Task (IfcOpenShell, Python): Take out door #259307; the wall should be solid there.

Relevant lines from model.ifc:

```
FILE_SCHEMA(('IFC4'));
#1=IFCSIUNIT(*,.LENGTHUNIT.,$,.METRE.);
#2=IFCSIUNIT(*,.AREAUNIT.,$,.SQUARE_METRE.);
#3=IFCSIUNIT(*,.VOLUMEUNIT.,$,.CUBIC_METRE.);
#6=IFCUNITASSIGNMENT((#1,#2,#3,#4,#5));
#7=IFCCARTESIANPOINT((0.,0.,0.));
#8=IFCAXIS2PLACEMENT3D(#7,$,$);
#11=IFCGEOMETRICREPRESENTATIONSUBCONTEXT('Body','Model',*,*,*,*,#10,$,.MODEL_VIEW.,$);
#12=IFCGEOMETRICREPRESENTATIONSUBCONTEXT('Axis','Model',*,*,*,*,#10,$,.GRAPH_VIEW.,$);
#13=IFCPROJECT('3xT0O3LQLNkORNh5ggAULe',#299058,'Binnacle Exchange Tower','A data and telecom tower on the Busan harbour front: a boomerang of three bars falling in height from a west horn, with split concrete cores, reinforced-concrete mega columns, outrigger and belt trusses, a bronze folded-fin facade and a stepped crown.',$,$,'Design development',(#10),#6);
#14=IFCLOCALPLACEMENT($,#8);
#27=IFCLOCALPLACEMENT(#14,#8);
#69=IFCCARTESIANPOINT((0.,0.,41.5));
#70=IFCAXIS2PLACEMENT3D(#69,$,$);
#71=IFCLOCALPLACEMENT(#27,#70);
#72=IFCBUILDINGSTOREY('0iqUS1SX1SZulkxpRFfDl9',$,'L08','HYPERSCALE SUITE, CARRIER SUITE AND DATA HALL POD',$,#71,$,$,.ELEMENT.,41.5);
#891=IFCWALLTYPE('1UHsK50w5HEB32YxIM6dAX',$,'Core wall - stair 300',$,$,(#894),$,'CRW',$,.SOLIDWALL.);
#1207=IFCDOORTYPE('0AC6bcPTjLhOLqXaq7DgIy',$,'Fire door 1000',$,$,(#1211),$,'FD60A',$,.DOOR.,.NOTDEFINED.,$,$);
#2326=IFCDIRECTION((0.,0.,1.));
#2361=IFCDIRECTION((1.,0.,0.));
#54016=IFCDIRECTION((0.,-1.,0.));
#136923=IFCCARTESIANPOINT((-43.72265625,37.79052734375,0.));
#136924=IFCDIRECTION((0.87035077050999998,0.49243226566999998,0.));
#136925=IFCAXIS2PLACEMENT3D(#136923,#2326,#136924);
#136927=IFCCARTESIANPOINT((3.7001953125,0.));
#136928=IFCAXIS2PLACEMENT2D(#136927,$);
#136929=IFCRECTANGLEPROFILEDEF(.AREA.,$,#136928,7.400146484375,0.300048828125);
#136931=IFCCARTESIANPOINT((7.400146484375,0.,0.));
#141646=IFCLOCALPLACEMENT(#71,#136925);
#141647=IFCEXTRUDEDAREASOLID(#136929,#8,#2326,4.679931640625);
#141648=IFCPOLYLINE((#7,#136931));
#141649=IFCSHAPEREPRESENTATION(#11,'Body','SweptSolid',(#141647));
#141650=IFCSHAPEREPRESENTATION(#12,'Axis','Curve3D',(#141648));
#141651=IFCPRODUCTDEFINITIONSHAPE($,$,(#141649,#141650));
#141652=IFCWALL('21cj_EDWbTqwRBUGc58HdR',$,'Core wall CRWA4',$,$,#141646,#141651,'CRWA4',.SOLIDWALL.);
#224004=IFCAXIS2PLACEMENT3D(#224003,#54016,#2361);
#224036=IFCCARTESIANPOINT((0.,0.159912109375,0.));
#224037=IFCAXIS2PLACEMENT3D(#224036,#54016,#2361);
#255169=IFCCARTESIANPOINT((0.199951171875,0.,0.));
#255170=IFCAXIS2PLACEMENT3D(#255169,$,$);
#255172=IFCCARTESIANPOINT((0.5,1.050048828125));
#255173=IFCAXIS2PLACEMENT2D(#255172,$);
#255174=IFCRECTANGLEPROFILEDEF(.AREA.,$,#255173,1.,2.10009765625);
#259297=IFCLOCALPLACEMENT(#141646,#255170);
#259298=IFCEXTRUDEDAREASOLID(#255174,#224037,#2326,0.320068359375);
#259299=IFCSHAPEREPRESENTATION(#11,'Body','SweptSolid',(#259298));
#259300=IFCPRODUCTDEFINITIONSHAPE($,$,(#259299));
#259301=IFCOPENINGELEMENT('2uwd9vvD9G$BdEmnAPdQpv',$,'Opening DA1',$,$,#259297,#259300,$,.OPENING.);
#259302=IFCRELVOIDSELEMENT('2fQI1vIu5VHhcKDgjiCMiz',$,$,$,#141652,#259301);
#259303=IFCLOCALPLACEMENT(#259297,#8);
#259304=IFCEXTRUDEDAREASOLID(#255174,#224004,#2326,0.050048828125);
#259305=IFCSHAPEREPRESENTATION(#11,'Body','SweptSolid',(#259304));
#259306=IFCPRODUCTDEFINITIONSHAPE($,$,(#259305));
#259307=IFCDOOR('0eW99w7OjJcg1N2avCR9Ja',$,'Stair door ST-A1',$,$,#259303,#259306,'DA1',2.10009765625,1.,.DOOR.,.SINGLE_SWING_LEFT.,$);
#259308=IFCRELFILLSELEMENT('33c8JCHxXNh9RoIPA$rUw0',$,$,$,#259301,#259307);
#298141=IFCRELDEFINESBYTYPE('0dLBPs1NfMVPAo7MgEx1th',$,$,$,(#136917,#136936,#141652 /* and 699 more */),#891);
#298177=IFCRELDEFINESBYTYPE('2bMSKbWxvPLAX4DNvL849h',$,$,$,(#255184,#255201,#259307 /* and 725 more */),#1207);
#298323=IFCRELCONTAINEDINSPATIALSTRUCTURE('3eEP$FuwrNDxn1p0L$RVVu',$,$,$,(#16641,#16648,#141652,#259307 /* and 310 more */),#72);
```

```python
import ifcopenshell
import ifcopenshell.api.feature
import ifcopenshell.api.root
import ifcopenshell.geom
import ifcopenshell.util.shape

model = ifcopenshell.open("model.ifc")
settings = ifcopenshell.geom.settings()


def volume(element):
    """Net volume in cubic metres, openings subtracted."""
    shape = ifcopenshell.geom.create_shape(settings, element)
    return ifcopenshell.util.shape.get_volume(shape.geometry)


door = model.by_id(259307)
opening = door.FillsVoids[0].RelatingOpeningElement
wall = opening.VoidsElements[0].RelatingBuildingElement
before = volume(wall)

ifcopenshell.api.root.remove_product(model, product=door)
ifcopenshell.api.feature.remove_feature(model, feature=opening)

after = volume(wall)

print(f"wall volume {before:.3f} -> {after:.3f} m3")

model.write("model_v2.ifc")
```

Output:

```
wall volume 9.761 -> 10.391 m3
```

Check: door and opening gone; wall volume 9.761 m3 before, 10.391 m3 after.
